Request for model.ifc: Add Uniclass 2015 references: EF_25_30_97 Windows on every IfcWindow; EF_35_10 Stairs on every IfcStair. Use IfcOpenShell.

First a look at what the model holds.

```python
import ifcopenshell

model = ifcopenshell.open("model.ifc")
print(model.schema)
print("classifications:", [c.Name for c in model.by_type("IfcClassification")])
for ifc_class in ("IfcDoor", "IfcRoof", "IfcStair", "IfcWall", "IfcWindow"):
    print(ifc_class, len(model.by_type(ifc_class)))
```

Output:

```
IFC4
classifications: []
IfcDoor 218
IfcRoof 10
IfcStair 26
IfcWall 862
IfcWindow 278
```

```python
import ifcopenshell
import ifcopenshell.api.classification

model = ifcopenshell.open("model.ifc")

system = ifcopenshell.api.classification.add_classification(model, classification="Uniclass 2015")

codes = {
    "IfcWindow": ("EF_25_30_97", "Windows"),
    "IfcStair": ("EF_35_10", "Stairs"),
}
for ifc_class, (code, name) in codes.items():
    products = model.by_type(ifc_class)
    ifcopenshell.api.classification.add_reference(
        model, products=products, classification=system, identification=code, name=name
    )
    print(code, len(products))

model.write("model_updated.ifc")
```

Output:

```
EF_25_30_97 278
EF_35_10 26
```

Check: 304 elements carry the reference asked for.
